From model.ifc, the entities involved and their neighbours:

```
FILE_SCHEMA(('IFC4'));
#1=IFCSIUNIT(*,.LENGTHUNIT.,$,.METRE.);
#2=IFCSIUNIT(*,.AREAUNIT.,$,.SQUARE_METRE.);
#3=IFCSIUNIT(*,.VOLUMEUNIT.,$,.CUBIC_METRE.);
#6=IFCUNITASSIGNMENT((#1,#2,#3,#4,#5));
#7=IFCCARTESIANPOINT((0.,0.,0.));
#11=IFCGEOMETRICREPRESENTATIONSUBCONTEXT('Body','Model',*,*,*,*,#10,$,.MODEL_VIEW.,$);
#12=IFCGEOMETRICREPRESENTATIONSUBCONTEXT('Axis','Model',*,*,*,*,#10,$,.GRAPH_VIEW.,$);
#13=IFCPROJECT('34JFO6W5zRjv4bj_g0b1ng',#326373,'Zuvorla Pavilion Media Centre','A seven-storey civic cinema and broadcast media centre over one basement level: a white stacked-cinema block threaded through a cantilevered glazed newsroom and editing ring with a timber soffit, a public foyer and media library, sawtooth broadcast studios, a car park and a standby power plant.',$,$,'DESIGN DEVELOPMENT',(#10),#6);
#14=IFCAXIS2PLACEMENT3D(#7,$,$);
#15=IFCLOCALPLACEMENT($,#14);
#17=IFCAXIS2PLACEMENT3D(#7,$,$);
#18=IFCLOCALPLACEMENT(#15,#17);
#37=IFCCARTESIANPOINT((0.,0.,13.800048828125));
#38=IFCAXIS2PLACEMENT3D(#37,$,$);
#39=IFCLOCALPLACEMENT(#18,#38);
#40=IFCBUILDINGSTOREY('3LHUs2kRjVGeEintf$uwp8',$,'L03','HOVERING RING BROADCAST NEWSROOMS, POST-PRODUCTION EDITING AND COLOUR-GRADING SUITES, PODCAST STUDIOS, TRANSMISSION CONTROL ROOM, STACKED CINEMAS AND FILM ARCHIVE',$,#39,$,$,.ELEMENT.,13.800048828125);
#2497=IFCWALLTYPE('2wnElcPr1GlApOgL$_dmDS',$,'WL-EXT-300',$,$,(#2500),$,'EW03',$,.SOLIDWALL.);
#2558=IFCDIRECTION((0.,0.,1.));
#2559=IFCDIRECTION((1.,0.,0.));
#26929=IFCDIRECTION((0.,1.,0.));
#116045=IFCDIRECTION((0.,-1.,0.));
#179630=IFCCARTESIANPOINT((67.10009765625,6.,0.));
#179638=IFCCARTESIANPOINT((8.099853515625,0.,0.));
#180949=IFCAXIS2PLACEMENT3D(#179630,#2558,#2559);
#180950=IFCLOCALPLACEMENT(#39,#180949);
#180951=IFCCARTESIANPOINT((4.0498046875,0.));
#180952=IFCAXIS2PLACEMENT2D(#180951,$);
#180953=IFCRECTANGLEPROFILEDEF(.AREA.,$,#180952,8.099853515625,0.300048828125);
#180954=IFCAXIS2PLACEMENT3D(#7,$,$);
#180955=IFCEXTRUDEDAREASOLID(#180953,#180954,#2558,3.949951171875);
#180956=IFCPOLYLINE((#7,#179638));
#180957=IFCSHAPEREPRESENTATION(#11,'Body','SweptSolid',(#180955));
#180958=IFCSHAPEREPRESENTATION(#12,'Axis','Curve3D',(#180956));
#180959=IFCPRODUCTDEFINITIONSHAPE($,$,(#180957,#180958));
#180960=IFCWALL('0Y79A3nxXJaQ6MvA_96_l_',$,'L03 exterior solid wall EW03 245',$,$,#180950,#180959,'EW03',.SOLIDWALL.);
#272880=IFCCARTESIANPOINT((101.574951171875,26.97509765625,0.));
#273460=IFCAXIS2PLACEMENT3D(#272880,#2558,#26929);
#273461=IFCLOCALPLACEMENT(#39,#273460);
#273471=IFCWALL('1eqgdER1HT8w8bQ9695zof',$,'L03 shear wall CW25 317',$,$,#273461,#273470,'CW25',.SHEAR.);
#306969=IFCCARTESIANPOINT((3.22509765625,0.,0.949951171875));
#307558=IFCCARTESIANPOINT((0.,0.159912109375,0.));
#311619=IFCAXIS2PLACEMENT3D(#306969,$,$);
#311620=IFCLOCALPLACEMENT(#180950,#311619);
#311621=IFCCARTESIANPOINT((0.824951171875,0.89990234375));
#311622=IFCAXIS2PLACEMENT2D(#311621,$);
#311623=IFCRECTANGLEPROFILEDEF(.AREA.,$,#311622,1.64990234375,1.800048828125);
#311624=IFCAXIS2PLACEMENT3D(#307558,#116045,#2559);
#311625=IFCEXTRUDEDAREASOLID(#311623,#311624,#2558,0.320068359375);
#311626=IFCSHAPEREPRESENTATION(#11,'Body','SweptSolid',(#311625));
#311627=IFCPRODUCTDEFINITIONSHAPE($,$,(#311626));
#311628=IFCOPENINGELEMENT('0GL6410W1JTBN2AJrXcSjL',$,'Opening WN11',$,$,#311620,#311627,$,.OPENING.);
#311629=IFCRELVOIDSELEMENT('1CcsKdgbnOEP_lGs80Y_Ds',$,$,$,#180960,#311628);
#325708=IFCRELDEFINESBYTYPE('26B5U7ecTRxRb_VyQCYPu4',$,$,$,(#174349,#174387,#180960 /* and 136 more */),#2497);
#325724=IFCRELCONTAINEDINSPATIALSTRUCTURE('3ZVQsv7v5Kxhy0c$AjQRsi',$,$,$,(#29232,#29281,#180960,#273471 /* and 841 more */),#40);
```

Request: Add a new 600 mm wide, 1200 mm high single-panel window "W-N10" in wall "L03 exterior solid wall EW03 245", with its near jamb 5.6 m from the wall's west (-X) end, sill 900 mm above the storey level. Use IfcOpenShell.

```python
import numpy as np
import ifcopenshell
import ifcopenshell.api.feature
import ifcopenshell.api.geometry
import ifcopenshell.api.root
import ifcopenshell.api.spatial
import ifcopenshell.geom
import ifcopenshell.util.element
import ifcopenshell.util.placement
import ifcopenshell.util.representation
import ifcopenshell.util.shape
import ifcopenshell.util.unit

model = ifcopenshell.open("model.ifc")
unit_scale = ifcopenshell.util.unit.calculate_unit_scale(model)
settings = ifcopenshell.geom.settings()


def volume(element):
    """Net volume in cubic metres, openings subtracted."""
    shape = ifcopenshell.geom.create_shape(settings, element)
    return ifcopenshell.util.shape.get_volume(shape.geometry)


wall = model.by_id(180960)
storey = ifcopenshell.util.element.get_container(wall, ifc_class="IfcBuildingStorey")
context = ifcopenshell.util.representation.get_context(model, "Model", "Body", "MODEL_VIEW")
before = volume(wall)

width, height, from_end, sill = 0.6, 1.2, 5.6, 0.9  # metres

# The wall runs along its own X axis, and the end named is its -X end.
wall_shape = ifcopenshell.geom.create_shape(settings, wall)
x, y, z = ifcopenshell.util.shape.get_vertices(wall_shape.geometry).T
start = x.min() + from_end
face, thickness = float(y.min()), float(y.max() - y.min())
wall_matrix = ifcopenshell.util.placement.get_local_placement(wall.ObjectPlacement)
level = ifcopenshell.util.placement.get_local_placement(storey.ObjectPlacement)[2, 3]


def in_wall(x, y):
    """Placement at x, y metres in the wall's axes, at sill height."""
    matrix = wall_matrix.copy()
    matrix[:, 3] = wall_matrix @ np.array([x / unit_scale, y / unit_scale, 0.0, 1.0])
    matrix[2, 3] = level + sill / unit_scale
    return matrix


# Opening: a box that overshoots both wall faces by 50 mm.
opening = ifcopenshell.api.root.create_entity(model, ifc_class="IfcOpeningElement", predefined_type="OPENING")
box = ifcopenshell.api.geometry.add_wall_representation(
    model, context=context, length=width, height=height, thickness=thickness + 0.1
)
ifcopenshell.api.geometry.assign_representation(model, product=opening, representation=box)
ifcopenshell.api.geometry.edit_object_placement(model, product=opening, matrix=in_wall(start, face - 0.05), is_si=False)
ifcopenshell.api.feature.add_feature(model, feature=opening, element=wall)

window = ifcopenshell.api.root.create_entity(model, ifc_class="IfcWindow", name="W-N10", predefined_type="WINDOW")
window.OverallWidth, window.OverallHeight = width / unit_scale, height / unit_scale
window.PartitioningType = "SINGLE_PANEL"
body = ifcopenshell.api.geometry.add_window_representation(
    model,
    context=context,
    overall_width=window.OverallWidth,
    overall_height=window.OverallHeight,
    partition_type="SINGLE_PANEL",
)
ifcopenshell.api.geometry.assign_representation(model, product=window, representation=body)
ifcopenshell.api.spatial.assign_container(model, products=[window], relating_structure=storey)
ifcopenshell.api.feature.add_filling(model, opening=opening, element=window)

# Centre the window in the wall's thickness.
ifcopenshell.api.geometry.edit_object_placement(model, product=window, matrix=in_wall(start, face), is_si=False)
window_shape = ifcopenshell.geom.create_shape(settings, window)
depth = ifcopenshell.util.shape.get_vertices(window_shape.geometry)[:, 1]
offset = face + thickness / 2 - (depth.min() + depth.max()) / 2
ifcopenshell.api.geometry.edit_object_placement(model, product=window, matrix=in_wall(start, offset), is_si=False)

after = volume(wall)

print(f"wall volume {before:.3f} -> {after:.3f} m3")

model.write("model_rev.ifc")
```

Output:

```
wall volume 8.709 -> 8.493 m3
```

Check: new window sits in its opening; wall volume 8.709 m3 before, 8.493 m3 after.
